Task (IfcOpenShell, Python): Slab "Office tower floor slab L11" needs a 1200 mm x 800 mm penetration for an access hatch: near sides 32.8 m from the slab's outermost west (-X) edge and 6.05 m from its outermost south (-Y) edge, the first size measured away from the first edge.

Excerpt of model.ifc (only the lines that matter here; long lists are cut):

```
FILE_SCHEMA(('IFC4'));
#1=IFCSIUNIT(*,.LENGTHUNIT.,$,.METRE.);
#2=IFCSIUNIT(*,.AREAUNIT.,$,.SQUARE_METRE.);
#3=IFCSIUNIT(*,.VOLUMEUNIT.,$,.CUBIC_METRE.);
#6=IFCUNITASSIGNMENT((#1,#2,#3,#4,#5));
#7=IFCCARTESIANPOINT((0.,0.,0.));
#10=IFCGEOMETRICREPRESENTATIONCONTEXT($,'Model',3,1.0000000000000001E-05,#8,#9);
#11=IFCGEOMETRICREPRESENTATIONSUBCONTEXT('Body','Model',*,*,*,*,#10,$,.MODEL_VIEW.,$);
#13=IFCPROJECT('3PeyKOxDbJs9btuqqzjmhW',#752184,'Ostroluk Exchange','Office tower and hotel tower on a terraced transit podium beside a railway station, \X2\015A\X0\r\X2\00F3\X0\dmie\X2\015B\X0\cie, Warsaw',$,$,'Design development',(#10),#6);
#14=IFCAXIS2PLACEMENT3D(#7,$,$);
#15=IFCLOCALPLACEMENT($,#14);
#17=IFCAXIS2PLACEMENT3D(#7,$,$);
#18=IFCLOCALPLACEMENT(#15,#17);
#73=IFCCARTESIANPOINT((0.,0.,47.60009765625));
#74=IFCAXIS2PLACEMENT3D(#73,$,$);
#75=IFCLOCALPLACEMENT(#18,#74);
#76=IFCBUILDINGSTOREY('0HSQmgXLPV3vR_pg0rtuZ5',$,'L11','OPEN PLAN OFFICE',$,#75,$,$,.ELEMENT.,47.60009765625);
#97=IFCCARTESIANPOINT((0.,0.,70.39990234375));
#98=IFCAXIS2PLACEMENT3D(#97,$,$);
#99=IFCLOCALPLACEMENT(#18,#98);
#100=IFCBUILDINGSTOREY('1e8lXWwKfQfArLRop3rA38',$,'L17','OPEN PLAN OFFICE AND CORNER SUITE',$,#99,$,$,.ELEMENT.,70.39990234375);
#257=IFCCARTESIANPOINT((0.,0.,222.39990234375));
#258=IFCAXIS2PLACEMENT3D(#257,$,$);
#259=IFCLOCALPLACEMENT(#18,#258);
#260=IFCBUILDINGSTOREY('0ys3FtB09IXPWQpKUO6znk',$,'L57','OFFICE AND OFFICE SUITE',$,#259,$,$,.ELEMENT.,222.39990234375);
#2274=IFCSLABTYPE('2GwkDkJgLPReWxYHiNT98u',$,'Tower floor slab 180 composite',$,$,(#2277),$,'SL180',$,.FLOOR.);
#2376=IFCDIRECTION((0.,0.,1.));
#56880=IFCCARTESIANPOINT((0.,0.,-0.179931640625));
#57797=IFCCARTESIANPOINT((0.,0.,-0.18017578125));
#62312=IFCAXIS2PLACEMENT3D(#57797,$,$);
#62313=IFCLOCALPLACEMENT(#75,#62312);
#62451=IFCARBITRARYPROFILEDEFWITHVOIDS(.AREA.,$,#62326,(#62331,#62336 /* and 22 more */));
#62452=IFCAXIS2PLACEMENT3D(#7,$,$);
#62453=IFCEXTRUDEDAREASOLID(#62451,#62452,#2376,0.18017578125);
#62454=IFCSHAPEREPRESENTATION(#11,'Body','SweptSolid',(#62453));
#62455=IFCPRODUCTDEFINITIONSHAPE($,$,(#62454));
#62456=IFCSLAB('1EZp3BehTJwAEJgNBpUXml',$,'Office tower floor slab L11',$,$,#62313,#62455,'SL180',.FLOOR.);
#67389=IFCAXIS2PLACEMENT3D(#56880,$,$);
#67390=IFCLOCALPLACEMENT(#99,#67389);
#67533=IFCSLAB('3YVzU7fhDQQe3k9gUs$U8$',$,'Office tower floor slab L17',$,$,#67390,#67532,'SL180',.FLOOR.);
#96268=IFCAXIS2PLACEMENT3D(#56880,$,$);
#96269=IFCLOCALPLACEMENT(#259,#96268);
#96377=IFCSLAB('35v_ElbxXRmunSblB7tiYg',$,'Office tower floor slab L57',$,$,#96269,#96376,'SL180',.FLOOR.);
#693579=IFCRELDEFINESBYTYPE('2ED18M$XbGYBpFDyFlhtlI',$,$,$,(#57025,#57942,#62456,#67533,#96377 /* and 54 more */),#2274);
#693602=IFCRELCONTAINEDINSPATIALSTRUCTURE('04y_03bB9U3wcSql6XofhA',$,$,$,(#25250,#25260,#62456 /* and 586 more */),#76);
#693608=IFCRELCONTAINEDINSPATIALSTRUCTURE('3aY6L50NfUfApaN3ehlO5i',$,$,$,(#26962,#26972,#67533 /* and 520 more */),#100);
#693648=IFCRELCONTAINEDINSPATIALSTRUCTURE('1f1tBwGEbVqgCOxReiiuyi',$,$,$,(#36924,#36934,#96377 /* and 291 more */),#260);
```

```python
import numpy as np
import ifcopenshell
import ifcopenshell.api.feature
import ifcopenshell.api.geometry
import ifcopenshell.api.root
import ifcopenshell.geom
import ifcopenshell.util.placement
import ifcopenshell.util.representation
import ifcopenshell.util.shape
import ifcopenshell.util.unit

model = ifcopenshell.open("model.ifc")
unit_scale = ifcopenshell.util.unit.calculate_unit_scale(model)
settings = ifcopenshell.geom.settings()


def volume(element):
    """Net volume in cubic metres, openings subtracted."""
    shape = ifcopenshell.geom.create_shape(settings, element)
    return ifcopenshell.util.shape.get_volume(shape.geometry)


slab = model.by_guid("1EZp3BehTJwAEJgNBpUXml")
before = volume(slab)

# Extent in the slab's own axes, in metres. The edges named are its -X and -Y sides.
slab_shape = ifcopenshell.geom.create_shape(settings, slab)
vertices = ifcopenshell.util.shape.get_vertices(slab_shape.geometry)
x_min, y_min, bottom = vertices.min(axis=0)
top = vertices[:, 2].max()

opening = ifcopenshell.api.root.create_entity(model, ifc_class="IfcOpeningElement", name="Access hatch opening", predefined_type="OPENING")
context = ifcopenshell.util.representation.get_context(model, "Model", "Body", "MODEL_VIEW")
width, depth = 1.2, 0.8
outline = [(0.0, 0.0), (width, 0.0), (width, depth), (0.0, depth), (0.0, 0.0)]
# Overshoot both faces by 50 mm so the cut is clean.
shape = ifcopenshell.api.geometry.add_slab_representation(
    model, context=context, depth=top - bottom + 0.1, polyline=outline
)
ifcopenshell.api.geometry.assign_representation(model, product=opening, representation=shape)

matrix = ifcopenshell.util.placement.get_local_placement(slab.ObjectPlacement)
matrix[:, 3] = matrix @ np.append(np.array([x_min + 32.8, y_min + 6.05, bottom - 0.05]) / unit_scale, 1.0)
ifcopenshell.api.geometry.edit_object_placement(model, product=opening, matrix=matrix, is_si=False)
ifcopenshell.api.feature.add_feature(model, feature=opening, element=slab)

after = volume(slab)

print(f"slab volume {before:.3f} -> {after:.3f} m3")

model.write("model_updated.ifc")
```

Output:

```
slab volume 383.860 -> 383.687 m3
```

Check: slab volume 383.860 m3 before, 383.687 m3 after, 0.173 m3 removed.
